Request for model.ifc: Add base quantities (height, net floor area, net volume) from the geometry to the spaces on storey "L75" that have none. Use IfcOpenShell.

First a look at what the model holds.

```python
import ifcopenshell
import ifcopenshell.util.element
import ifcopenshell.util.unit

model = ifcopenshell.open("model.ifc")
print(model.schema)
for unit_type in ("LENGTHUNIT", "AREAUNIT", "VOLUMEUNIT"):
    print(unit_type, ifcopenshell.util.unit.calculate_unit_scale(model, unit_type))
storey = next(s for s in model.by_type("IfcBuildingStorey") if s.Name == "L75")
spaces = [e for e in ifcopenshell.util.element.get_decomposition(storey) if e.is_a("IfcSpace")]
for e in sorted(spaces, key=lambda e: e.id()):
    print(e.id(), e.is_a(), e.Name, list(ifcopenshell.util.element.get_psets(e, qtos_only=True)), sep=" | ")
```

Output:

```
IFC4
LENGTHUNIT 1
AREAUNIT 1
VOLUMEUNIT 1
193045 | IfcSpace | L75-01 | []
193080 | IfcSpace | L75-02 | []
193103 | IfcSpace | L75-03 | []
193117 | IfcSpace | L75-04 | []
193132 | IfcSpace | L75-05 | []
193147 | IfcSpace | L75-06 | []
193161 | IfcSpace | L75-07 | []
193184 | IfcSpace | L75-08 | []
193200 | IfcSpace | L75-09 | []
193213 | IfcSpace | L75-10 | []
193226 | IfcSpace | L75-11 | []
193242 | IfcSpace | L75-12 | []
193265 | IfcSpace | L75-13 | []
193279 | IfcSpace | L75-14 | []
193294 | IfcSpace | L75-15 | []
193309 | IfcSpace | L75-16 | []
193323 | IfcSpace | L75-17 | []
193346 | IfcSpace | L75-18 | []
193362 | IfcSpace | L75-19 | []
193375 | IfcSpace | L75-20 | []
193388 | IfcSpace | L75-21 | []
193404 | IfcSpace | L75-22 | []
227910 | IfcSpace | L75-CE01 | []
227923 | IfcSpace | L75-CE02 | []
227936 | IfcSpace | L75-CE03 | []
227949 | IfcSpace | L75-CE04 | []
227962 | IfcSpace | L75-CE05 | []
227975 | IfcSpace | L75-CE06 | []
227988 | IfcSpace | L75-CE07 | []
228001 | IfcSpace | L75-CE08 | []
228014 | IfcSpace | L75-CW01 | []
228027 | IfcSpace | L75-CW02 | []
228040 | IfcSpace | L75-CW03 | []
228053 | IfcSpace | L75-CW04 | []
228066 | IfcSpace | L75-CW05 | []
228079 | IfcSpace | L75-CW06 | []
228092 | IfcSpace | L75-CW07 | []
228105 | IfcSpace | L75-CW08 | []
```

```python
import ifcopenshell
import ifcopenshell.api.pset
import ifcopenshell.geom
import ifcopenshell.util.element
import ifcopenshell.util.shape
import ifcopenshell.util.unit

model = ifcopenshell.open("model.ifc")
unit_scale = ifcopenshell.util.unit.calculate_unit_scale(model)
area_scale = ifcopenshell.util.unit.calculate_unit_scale(model, "AREAUNIT")
volume_scale = ifcopenshell.util.unit.calculate_unit_scale(model, "VOLUMEUNIT")
settings = ifcopenshell.geom.settings()

storey = next(s for s in model.by_type("IfcBuildingStorey") if s.Name == "L75")
spaces = [e for e in ifcopenshell.util.element.get_decomposition(storey) if e.is_a("IfcSpace")]

for e in sorted(spaces, key=lambda e: e.id()):
    if ifcopenshell.util.element.get_psets(e, qtos_only=True, should_inherit=False):
        continue
    # Geometry comes back in metres, in the element's own axes.
    shape = ifcopenshell.geom.create_shape(settings, e)
    values = {
        "Height": ifcopenshell.util.shape.get_z(shape.geometry) / unit_scale,
        "NetFloorArea": ifcopenshell.util.shape.get_footprint_area(shape.geometry) / area_scale,
        "NetVolume": ifcopenshell.util.shape.get_volume(shape.geometry) / volume_scale,
    }
    qto = ifcopenshell.api.pset.add_qto(model, product=e, name="Qto_SpaceBaseQuantities")
    ifcopenshell.api.pset.edit_qto(model, qto=qto, properties=values)
    print(e.id(), {k: round(v, 3) for k, v in values.items()})

model.write("model_edited.ifc")
```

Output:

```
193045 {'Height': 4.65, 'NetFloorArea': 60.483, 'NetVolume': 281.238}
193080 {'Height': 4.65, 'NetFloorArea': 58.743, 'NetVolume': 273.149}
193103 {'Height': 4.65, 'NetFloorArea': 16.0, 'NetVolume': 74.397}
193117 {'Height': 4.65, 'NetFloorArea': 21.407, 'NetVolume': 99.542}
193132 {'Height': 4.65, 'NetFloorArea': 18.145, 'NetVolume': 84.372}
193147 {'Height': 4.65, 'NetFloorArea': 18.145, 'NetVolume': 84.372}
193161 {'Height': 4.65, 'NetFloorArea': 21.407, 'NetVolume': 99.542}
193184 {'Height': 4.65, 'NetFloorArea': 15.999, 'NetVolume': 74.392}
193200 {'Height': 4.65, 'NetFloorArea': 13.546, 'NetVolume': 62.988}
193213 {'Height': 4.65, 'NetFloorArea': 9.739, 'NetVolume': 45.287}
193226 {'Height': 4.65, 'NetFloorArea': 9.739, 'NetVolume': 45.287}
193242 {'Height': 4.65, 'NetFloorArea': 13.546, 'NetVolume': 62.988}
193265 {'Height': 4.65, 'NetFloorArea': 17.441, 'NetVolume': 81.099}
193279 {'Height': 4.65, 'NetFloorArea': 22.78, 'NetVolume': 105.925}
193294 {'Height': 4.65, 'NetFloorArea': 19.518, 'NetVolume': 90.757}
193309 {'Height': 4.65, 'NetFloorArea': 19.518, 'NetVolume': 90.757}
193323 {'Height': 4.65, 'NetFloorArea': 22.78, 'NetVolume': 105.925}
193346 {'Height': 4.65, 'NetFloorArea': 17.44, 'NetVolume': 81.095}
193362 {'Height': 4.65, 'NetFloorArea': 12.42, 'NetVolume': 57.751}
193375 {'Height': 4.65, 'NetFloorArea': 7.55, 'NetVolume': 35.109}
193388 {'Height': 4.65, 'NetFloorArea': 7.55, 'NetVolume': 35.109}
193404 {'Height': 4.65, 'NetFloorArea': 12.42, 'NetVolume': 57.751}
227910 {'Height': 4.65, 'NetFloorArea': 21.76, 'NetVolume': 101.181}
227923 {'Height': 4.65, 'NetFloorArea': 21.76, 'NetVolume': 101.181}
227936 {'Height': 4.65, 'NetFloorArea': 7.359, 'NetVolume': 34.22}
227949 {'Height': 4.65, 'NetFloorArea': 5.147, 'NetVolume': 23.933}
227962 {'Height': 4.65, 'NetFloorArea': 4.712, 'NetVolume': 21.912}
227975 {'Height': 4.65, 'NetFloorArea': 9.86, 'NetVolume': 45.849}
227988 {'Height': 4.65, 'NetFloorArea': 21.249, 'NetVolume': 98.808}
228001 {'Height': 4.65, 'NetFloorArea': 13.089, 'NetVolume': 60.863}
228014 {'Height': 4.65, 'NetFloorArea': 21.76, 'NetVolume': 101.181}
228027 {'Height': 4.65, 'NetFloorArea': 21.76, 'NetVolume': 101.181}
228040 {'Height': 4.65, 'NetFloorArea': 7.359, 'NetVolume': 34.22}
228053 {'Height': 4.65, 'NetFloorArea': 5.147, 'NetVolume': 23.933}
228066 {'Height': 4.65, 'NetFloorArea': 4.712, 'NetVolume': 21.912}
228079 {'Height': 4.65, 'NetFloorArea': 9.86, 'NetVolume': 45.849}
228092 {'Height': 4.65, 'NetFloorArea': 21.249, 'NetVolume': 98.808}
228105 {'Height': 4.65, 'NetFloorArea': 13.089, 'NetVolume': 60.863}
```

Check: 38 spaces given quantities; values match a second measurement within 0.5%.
